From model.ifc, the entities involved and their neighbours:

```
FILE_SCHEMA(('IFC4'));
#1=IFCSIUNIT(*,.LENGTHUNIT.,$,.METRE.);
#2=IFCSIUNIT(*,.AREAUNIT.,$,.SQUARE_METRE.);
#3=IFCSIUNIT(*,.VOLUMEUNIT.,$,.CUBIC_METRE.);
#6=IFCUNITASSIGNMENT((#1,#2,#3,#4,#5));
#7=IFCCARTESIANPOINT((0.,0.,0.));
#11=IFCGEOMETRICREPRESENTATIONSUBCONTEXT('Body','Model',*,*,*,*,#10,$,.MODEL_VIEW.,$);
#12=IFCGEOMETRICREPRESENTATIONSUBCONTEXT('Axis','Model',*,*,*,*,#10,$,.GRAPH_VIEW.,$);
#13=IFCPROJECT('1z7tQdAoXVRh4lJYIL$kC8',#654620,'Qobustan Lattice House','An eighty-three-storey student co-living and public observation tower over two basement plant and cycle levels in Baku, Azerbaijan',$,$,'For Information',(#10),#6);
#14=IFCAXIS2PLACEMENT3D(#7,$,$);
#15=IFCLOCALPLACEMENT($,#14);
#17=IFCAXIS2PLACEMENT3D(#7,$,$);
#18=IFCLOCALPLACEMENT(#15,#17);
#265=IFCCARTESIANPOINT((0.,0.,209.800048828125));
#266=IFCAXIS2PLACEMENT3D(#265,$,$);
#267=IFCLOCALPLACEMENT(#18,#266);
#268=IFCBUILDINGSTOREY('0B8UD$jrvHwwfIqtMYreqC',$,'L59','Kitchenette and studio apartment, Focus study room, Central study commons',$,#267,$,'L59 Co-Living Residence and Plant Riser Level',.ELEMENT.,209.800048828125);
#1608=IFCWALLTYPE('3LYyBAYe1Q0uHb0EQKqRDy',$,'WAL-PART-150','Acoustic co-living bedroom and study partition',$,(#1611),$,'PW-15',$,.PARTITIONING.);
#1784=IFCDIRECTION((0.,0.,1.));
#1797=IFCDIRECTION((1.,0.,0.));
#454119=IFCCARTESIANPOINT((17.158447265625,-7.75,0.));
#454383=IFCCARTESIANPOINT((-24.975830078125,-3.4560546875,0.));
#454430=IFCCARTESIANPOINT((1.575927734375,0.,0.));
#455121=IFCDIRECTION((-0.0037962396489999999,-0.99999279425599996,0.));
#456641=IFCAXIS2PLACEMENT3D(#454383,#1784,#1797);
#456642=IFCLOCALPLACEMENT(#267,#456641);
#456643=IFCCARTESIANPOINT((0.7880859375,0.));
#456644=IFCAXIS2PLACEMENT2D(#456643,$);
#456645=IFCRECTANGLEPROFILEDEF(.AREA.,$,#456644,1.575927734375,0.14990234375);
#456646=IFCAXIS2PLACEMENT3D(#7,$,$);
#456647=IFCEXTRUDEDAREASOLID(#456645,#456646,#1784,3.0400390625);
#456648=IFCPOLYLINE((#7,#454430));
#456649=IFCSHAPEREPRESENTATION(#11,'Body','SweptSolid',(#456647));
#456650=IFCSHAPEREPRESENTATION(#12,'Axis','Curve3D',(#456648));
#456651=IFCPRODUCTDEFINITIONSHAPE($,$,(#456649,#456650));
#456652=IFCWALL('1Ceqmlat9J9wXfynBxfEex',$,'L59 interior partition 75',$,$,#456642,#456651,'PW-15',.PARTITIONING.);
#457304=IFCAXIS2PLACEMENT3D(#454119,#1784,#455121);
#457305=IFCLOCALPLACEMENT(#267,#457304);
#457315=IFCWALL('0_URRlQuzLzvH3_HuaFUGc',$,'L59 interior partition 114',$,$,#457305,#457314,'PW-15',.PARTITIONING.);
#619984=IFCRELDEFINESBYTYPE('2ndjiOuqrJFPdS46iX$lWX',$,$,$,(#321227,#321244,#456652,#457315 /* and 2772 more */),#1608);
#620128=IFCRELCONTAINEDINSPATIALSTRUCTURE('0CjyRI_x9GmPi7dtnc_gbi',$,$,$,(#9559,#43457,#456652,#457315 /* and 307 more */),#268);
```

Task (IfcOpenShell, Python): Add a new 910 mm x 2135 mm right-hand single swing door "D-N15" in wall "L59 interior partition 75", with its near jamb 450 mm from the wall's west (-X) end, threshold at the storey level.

```python
import numpy as np
import ifcopenshell
import ifcopenshell.api.feature
import ifcopenshell.api.geometry
import ifcopenshell.api.root
import ifcopenshell.api.spatial
import ifcopenshell.geom
import ifcopenshell.util.element
import ifcopenshell.util.placement
import ifcopenshell.util.representation
import ifcopenshell.util.shape
import ifcopenshell.util.unit

model = ifcopenshell.open("model.ifc")
unit_scale = ifcopenshell.util.unit.calculate_unit_scale(model)
settings = ifcopenshell.geom.settings()


def volume(element):
    """Net volume in cubic metres, openings subtracted."""
    shape = ifcopenshell.geom.create_shape(settings, element)
    return ifcopenshell.util.shape.get_volume(shape.geometry)


wall = model.by_guid("1Ceqmlat9J9wXfynBxfEex")
storey = ifcopenshell.util.element.get_container(wall, ifc_class="IfcBuildingStorey")
context = ifcopenshell.util.representation.get_context(model, "Model", "Body", "MODEL_VIEW")
before = volume(wall)

width, height, from_end, sill = 0.91, 2.135, 0.45, 0.0  # metres

# The wall runs along its own X axis, and the end named is its -X end.
wall_shape = ifcopenshell.geom.create_shape(settings, wall)
x, y, z = ifcopenshell.util.shape.get_vertices(wall_shape.geometry).T
start = x.min() + from_end
face, thickness = float(y.min()), float(y.max() - y.min())
wall_matrix = ifcopenshell.util.placement.get_local_placement(wall.ObjectPlacement)
level = ifcopenshell.util.placement.get_local_placement(storey.ObjectPlacement)[2, 3]


def in_wall(x, y):
    """Placement at x, y metres in the wall's axes, at sill height."""
    matrix = wall_matrix.copy()
    matrix[:, 3] = wall_matrix @ np.array([x / unit_scale, y / unit_scale, 0.0, 1.0])
    matrix[2, 3] = level + sill / unit_scale
    return matrix


# Opening: a box that overshoots both wall faces by 50 mm.
opening = ifcopenshell.api.root.create_entity(model, ifc_class="IfcOpeningElement", predefined_type="OPENING")
box = ifcopenshell.api.geometry.add_wall_representation(
    model, context=context, length=width, height=height, thickness=thickness + 0.1
)
ifcopenshell.api.geometry.assign_representation(model, product=opening, representation=box)
ifcopenshell.api.geometry.edit_object_placement(model, product=opening, matrix=in_wall(start, face - 0.05), is_si=False)
ifcopenshell.api.feature.add_feature(model, feature=opening, element=wall)

door = ifcopenshell.api.root.create_entity(model, ifc_class="IfcDoor", name="D-N15", predefined_type="DOOR")
door.OverallWidth, door.OverallHeight = width / unit_scale, height / unit_scale
door.OperationType = "SINGLE_SWING_RIGHT"
body = ifcopenshell.api.geometry.add_door_representation(
    model,
    context=context,
    overall_width=door.OverallWidth,
    overall_height=door.OverallHeight,
    operation_type="SINGLE_SWING_RIGHT",
    lining_properties={"LiningDepth": thickness / unit_scale, "ThresholdDepth": thickness / unit_scale},
)
ifcopenshell.api.geometry.assign_representation(model, product=door, representation=body)
ifcopenshell.api.spatial.assign_container(model, products=[door], relating_structure=storey)
ifcopenshell.api.feature.add_filling(model, opening=opening, element=door)

# The lining spans the wall, so the door starts at the wall face.
ifcopenshell.api.geometry.edit_object_placement(model, product=door, matrix=in_wall(start, face), is_si=False)

after = volume(wall)

print(f"wall volume {before:.3f} -> {after:.3f} m3")

model.write("model-out.ifc")
```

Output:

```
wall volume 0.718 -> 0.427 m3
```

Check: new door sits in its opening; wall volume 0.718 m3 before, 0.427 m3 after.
